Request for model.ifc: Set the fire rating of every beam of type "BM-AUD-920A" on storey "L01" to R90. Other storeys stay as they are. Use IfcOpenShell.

First a look at what the model holds.

```python
import ifcopenshell
import ifcopenshell.util.element

model = ifcopenshell.open("model.ifc")
print(model.schema)
storey = next(s for s in model.by_type("IfcBuildingStorey") if s.Name == "L01")
beams = [e for e in ifcopenshell.util.element.get_decomposition(storey) if e.is_a("IfcBeam")]
seen = {}
for e in beams:
    element_type = ifcopenshell.util.element.get_type(e)
    key = (element_type.Name if element_type != e and element_type else None, ifcopenshell.util.element.get_pset(e, "Pset_BeamCommon", "FireRating"))
    seen[key] = seen.get(key, 0) + 1
for (name, value), count in sorted(seen.items(), key=str):
    print(count, "x", name, "|", value)
```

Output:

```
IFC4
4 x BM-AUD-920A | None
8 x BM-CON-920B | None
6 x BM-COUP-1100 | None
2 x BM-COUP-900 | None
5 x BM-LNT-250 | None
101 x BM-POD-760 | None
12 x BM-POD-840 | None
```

```python
import ifcopenshell
import ifcopenshell.api.pset
import ifcopenshell.util.element

model = ifcopenshell.open("model.ifc")

storey = next(s for s in model.by_type("IfcBuildingStorey") if s.Name == "L01")
beams = [e for e in ifcopenshell.util.element.get_decomposition(storey) if e.is_a("IfcBeam")]

count = 0
for e in beams:
    element_type = ifcopenshell.util.element.get_type(e)
    if element_type in (None, e) or element_type.Name != "BM-AUD-920A":
        continue
    found = ifcopenshell.util.element.get_pset(e, "Pset_BeamCommon", should_inherit=False)
    if found:
        pset = model.by_id(found["id"])
        if len(ifcopenshell.util.element.get_elements_by_pset(pset)) > 1:
            pset = ifcopenshell.api.pset.unshare_pset(model, products=[e], pset=pset)[0]
    else:
        pset = ifcopenshell.api.pset.add_pset(model, product=e, name="Pset_BeamCommon")
    ifcopenshell.api.pset.edit_pset(model, pset=pset, properties={"FireRating": "R90"})
    count += 1

print(count, "beams updated")

model.write("model_rev.ifc")
```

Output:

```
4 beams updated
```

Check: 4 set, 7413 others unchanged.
